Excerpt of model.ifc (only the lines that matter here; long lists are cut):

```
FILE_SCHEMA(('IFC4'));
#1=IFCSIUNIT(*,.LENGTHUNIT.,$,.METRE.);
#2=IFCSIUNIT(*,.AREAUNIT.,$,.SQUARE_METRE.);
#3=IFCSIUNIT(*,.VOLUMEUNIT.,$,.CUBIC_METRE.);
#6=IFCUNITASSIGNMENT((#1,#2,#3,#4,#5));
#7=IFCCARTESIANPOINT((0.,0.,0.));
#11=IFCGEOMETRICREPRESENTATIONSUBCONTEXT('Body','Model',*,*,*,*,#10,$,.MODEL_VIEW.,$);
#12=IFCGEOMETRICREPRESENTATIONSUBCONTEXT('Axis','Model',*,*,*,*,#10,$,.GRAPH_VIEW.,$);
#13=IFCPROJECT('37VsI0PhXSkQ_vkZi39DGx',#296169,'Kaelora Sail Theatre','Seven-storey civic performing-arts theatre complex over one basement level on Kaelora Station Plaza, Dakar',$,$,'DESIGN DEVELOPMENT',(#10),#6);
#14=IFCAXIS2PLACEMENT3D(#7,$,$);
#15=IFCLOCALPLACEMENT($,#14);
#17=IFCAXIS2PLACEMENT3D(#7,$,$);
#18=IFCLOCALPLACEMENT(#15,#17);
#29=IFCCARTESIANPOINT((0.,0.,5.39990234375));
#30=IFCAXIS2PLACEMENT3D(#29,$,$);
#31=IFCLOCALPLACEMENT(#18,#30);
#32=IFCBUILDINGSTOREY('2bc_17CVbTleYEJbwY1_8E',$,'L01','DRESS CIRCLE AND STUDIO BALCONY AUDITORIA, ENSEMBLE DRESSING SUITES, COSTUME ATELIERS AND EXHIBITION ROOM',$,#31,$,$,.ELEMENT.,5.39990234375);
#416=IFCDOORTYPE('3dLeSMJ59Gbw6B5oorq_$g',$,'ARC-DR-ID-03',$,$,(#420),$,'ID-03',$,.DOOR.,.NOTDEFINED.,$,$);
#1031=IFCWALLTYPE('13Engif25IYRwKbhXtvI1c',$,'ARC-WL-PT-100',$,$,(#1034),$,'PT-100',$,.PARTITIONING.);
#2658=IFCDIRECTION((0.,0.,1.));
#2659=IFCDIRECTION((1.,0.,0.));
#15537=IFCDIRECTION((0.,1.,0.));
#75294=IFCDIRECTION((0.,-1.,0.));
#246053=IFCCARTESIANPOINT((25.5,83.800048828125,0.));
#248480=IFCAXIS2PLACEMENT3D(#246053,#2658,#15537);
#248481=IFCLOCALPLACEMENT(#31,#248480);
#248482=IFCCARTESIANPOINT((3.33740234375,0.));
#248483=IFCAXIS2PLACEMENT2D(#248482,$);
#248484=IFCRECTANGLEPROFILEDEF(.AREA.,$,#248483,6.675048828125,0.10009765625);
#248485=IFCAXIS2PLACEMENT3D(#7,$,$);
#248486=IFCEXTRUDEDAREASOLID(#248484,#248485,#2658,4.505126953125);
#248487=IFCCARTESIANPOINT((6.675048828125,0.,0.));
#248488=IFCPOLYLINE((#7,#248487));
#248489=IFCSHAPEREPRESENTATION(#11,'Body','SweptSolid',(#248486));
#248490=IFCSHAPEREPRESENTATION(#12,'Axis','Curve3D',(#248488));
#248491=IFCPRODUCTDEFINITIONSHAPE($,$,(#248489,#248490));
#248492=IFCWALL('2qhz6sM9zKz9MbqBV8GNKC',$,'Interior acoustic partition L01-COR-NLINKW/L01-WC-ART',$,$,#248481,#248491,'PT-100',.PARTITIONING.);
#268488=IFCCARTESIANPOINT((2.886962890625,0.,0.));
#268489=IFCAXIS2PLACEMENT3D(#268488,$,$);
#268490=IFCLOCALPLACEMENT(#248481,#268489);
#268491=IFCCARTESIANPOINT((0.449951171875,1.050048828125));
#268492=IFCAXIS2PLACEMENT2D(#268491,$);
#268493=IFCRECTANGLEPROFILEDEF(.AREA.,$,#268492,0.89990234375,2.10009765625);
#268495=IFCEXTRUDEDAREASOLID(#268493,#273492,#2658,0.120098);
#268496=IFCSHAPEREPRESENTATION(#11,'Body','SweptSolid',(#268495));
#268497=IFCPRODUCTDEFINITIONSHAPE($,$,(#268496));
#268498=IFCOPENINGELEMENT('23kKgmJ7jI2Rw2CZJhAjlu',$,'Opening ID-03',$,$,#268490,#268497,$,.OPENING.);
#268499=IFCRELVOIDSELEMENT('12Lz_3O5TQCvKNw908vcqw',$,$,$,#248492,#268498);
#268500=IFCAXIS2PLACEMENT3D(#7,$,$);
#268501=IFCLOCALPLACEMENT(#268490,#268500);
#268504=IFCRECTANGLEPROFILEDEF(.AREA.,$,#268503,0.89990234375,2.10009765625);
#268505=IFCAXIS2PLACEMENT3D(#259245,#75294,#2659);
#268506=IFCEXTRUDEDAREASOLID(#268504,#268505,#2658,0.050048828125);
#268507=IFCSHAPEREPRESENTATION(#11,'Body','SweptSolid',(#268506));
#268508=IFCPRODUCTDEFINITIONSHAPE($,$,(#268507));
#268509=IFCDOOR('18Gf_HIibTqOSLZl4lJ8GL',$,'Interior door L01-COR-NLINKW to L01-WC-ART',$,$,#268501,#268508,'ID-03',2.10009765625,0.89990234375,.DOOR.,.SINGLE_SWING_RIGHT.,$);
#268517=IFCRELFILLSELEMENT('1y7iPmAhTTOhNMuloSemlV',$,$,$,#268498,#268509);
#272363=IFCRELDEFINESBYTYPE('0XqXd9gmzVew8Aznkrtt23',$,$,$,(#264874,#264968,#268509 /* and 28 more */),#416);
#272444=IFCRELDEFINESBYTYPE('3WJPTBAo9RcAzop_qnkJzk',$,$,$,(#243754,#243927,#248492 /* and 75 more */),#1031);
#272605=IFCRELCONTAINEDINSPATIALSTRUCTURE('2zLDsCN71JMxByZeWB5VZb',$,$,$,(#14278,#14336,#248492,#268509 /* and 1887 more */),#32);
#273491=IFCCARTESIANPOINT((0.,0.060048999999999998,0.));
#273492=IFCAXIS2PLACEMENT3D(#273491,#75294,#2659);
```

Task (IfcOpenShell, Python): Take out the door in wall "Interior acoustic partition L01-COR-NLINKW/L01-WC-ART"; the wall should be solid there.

```python
import ifcopenshell
import ifcopenshell.api.feature
import ifcopenshell.api.root
import ifcopenshell.geom
import ifcopenshell.util.shape

model = ifcopenshell.open("model.ifc")
settings = ifcopenshell.geom.settings()


def volume(element):
    """Net volume in cubic metres, openings subtracted."""
    shape = ifcopenshell.geom.create_shape(settings, element)
    return ifcopenshell.util.shape.get_volume(shape.geometry)


door = model.by_id(268509)
opening = door.FillsVoids[0].RelatingOpeningElement
wall = opening.VoidsElements[0].RelatingBuildingElement
before = volume(wall)

ifcopenshell.api.root.remove_product(model, product=door)
ifcopenshell.api.feature.remove_feature(model, feature=opening)

after = volume(wall)

print(f"wall volume {before:.3f} -> {after:.3f} m3")

model.write("model_updated.ifc")
```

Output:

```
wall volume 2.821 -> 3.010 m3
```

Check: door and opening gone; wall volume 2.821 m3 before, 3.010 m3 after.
